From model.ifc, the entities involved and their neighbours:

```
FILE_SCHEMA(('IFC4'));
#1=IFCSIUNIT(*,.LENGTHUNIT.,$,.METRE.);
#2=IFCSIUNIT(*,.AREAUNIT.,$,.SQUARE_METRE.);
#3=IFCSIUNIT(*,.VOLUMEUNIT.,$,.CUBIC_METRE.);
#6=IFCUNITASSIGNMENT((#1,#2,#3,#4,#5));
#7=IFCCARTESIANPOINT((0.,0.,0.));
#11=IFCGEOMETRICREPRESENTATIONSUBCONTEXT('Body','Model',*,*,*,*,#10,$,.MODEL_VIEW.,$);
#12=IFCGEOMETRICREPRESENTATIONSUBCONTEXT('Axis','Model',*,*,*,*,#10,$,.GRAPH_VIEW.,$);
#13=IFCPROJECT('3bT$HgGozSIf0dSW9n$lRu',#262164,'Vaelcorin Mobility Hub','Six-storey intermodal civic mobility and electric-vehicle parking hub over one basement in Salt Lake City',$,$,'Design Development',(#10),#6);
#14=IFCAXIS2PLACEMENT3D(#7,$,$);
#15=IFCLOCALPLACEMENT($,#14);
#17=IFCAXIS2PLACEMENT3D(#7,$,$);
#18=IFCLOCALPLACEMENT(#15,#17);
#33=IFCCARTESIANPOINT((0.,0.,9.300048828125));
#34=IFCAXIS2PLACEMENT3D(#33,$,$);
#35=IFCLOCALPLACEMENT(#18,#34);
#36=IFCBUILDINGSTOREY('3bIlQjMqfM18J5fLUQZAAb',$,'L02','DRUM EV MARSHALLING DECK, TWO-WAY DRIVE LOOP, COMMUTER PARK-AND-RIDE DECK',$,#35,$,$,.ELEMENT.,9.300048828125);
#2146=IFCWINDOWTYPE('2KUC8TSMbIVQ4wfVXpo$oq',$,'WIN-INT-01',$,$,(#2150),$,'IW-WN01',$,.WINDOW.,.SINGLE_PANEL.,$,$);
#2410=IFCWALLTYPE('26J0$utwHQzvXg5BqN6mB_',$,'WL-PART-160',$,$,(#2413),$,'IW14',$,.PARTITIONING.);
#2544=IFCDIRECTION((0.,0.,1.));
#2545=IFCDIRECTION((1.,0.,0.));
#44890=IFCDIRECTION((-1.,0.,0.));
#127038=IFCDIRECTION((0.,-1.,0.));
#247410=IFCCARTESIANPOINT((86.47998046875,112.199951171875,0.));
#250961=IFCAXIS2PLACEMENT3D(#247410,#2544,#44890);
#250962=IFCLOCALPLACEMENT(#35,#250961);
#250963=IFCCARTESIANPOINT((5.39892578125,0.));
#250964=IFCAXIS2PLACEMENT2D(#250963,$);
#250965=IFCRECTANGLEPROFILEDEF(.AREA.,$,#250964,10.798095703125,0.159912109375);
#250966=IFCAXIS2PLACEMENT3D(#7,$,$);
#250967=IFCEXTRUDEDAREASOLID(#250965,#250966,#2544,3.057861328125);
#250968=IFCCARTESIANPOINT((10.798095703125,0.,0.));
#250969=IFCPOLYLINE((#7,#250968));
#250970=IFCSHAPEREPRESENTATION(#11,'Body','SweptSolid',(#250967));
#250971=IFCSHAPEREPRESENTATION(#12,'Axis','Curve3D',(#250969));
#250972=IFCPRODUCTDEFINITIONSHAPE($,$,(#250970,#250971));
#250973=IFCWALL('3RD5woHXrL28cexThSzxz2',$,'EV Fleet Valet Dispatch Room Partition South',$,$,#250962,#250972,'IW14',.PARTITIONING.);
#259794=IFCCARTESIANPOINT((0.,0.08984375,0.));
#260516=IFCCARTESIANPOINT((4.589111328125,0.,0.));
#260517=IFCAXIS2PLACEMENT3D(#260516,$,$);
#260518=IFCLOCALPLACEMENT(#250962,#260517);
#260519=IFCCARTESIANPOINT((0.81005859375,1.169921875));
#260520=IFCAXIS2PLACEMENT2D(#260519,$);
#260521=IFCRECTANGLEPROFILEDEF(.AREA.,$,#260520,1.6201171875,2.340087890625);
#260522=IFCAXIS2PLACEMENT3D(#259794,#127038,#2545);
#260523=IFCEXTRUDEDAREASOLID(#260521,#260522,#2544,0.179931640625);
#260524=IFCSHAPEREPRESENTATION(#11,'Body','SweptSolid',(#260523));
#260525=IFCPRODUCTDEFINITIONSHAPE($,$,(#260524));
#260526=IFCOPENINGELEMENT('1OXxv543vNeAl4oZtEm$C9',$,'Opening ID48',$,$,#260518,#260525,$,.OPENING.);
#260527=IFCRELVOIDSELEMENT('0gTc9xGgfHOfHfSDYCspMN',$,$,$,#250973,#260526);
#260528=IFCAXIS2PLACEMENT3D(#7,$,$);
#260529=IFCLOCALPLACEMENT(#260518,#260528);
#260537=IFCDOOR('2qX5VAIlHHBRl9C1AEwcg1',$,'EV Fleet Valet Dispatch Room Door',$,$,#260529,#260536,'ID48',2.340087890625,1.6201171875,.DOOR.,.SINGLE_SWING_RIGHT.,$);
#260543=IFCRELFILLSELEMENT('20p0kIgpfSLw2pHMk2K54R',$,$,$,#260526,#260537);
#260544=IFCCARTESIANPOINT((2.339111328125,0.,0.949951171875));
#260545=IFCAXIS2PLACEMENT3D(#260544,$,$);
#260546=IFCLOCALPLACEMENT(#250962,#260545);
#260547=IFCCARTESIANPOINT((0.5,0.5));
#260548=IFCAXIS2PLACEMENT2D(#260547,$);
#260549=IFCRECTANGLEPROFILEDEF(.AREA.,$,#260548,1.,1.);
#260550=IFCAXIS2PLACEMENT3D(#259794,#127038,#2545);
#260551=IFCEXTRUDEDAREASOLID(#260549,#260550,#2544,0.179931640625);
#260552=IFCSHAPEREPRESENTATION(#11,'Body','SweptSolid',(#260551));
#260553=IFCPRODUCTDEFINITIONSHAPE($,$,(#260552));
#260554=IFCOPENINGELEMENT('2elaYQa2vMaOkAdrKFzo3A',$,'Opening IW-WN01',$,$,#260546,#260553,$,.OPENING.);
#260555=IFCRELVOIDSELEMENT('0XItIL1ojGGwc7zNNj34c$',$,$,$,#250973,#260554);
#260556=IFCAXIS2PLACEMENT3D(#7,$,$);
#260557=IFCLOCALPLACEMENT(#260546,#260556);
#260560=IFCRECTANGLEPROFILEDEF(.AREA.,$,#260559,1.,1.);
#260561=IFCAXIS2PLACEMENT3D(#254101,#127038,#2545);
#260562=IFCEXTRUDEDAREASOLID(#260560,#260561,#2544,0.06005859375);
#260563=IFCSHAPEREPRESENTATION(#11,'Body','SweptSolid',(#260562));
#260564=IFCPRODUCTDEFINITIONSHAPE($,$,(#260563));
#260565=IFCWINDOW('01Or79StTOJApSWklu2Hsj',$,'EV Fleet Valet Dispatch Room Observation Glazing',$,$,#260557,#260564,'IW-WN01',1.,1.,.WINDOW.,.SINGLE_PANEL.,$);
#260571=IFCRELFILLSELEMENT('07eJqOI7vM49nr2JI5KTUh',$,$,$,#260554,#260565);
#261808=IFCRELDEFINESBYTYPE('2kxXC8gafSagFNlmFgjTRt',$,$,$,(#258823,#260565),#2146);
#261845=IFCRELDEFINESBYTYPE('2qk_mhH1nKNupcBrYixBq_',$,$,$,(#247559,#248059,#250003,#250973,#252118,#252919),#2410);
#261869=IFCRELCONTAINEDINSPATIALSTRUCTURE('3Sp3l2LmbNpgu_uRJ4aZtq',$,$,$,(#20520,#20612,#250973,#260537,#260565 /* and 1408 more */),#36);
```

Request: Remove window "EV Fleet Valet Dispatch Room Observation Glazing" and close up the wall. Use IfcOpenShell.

```python
import ifcopenshell
import ifcopenshell.api.feature
import ifcopenshell.api.root
import ifcopenshell.geom
import ifcopenshell.util.shape

model = ifcopenshell.open("model.ifc")
settings = ifcopenshell.geom.settings()


def volume(element):
    """Net volume in cubic metres, openings subtracted."""
    shape = ifcopenshell.geom.create_shape(settings, element)
    return ifcopenshell.util.shape.get_volume(shape.geometry)


window = model.by_id(260565)
opening = window.FillsVoids[0].RelatingOpeningElement
wall = opening.VoidsElements[0].RelatingBuildingElement
before = volume(wall)

ifcopenshell.api.root.remove_product(model, product=window)
ifcopenshell.api.feature.remove_feature(model, feature=opening)

after = volume(wall)

print(f"wall volume {before:.3f} -> {after:.3f} m3")

model.write("model_v2.ifc")
```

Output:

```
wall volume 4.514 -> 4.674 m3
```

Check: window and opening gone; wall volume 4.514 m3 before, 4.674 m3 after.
